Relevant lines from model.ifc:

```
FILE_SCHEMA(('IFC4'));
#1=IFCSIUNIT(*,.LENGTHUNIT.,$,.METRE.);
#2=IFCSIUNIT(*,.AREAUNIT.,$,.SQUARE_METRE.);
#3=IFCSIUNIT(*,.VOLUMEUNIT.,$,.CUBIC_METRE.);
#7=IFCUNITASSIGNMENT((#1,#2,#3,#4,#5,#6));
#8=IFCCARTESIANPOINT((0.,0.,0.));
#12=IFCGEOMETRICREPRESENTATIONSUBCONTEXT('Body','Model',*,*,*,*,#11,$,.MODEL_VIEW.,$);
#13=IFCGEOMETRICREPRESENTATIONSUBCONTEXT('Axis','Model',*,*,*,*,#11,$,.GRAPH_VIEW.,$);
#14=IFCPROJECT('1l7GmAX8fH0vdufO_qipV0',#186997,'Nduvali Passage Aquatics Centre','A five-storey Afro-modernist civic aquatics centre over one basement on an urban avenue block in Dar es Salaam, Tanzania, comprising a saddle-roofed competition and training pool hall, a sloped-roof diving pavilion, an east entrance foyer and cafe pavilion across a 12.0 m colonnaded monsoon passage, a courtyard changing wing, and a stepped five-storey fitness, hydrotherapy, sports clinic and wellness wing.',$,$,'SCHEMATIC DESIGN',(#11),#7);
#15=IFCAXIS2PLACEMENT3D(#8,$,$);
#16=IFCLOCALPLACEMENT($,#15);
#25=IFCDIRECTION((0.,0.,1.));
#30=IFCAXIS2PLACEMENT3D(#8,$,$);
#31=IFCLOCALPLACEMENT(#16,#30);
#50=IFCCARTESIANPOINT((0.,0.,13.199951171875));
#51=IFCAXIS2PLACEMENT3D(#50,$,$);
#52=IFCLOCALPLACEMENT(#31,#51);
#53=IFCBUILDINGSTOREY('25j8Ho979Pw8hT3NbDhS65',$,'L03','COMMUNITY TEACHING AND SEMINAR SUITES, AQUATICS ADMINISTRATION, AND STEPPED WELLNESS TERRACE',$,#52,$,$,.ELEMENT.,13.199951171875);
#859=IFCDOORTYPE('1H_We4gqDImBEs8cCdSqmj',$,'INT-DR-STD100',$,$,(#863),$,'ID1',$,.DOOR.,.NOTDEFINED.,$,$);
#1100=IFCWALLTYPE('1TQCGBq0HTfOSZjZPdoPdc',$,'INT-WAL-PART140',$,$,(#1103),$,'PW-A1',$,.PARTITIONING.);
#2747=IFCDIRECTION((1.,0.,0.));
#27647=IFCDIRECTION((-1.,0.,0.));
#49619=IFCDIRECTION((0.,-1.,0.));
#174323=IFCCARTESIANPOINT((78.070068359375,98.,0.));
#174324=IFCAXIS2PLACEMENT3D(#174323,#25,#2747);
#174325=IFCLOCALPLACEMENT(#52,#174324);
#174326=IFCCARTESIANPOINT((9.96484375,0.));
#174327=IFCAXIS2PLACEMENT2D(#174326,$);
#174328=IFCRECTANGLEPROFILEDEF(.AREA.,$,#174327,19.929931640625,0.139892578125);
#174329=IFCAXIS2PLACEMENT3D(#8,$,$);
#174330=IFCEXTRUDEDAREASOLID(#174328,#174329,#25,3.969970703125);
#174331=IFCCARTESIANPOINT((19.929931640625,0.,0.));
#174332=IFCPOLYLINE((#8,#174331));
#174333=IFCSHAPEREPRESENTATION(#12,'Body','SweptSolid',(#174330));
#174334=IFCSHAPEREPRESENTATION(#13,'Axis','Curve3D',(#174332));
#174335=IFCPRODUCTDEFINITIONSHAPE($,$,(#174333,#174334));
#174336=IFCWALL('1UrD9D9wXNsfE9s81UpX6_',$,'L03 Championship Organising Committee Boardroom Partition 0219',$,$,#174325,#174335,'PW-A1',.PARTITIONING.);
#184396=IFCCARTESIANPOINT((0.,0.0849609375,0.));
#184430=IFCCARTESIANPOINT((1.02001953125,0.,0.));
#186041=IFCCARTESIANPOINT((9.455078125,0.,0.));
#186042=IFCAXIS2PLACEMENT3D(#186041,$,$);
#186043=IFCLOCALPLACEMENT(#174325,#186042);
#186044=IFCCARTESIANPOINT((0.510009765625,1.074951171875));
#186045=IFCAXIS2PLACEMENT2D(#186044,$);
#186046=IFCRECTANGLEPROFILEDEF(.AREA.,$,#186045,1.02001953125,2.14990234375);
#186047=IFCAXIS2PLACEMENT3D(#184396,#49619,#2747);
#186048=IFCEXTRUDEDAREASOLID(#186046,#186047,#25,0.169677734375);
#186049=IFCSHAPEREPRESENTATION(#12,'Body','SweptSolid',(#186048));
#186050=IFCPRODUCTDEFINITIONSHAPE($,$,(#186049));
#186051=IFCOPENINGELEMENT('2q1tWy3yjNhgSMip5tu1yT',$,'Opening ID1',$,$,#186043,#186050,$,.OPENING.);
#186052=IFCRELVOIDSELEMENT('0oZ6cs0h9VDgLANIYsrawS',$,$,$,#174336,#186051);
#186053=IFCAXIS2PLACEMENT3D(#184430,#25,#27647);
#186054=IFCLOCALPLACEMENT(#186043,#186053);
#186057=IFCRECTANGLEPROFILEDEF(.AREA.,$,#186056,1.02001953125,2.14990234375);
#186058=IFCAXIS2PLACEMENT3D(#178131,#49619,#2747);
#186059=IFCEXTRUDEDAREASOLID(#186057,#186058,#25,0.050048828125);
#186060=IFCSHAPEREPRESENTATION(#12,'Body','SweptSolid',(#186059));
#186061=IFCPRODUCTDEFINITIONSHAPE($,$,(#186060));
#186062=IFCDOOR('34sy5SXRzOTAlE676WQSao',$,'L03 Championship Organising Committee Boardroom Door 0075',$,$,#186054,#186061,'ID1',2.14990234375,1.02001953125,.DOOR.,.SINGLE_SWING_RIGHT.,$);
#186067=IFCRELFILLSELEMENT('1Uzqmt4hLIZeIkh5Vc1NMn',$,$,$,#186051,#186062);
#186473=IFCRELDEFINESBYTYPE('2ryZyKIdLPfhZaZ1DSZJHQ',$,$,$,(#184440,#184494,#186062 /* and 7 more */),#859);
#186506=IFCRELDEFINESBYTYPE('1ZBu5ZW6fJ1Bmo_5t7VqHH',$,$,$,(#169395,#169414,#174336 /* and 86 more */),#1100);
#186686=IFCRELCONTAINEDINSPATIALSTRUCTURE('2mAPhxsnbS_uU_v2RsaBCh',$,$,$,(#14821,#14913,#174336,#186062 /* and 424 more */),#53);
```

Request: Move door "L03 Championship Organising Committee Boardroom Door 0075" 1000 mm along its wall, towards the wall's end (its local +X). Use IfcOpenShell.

```python
import ifcopenshell
import ifcopenshell.api.geometry
import ifcopenshell.util.placement

model = ifcopenshell.open("model.ifc")

door = model.by_guid("34sy5SXRzOTAlE676WQSao")
opening = door.FillsVoids[0].RelatingOpeningElement
wall = opening.VoidsElements[0].RelatingBuildingElement

wall_matrix = ifcopenshell.util.placement.get_local_placement(wall.ObjectPlacement)
shift = wall_matrix[:3, 0] * 1.0
before = ifcopenshell.util.placement.get_local_placement(door.ObjectPlacement)[:3, 3].copy()

# The door is placed relative to its opening, so it follows when the opening moves.
matrix = ifcopenshell.util.placement.get_local_placement(opening.ObjectPlacement)
matrix[:3, 3] += shift
ifcopenshell.api.geometry.edit_object_placement(
    model, product=opening, matrix=matrix, is_si=False, should_transform_children=True
)

after = ifcopenshell.util.placement.get_local_placement(door.ObjectPlacement)[:3, 3]
print("door moved by", (after - before).round(3) + 0.0)

model.write("model_rev.ifc")
```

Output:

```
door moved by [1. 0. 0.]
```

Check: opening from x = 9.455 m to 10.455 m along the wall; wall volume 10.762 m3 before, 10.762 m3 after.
